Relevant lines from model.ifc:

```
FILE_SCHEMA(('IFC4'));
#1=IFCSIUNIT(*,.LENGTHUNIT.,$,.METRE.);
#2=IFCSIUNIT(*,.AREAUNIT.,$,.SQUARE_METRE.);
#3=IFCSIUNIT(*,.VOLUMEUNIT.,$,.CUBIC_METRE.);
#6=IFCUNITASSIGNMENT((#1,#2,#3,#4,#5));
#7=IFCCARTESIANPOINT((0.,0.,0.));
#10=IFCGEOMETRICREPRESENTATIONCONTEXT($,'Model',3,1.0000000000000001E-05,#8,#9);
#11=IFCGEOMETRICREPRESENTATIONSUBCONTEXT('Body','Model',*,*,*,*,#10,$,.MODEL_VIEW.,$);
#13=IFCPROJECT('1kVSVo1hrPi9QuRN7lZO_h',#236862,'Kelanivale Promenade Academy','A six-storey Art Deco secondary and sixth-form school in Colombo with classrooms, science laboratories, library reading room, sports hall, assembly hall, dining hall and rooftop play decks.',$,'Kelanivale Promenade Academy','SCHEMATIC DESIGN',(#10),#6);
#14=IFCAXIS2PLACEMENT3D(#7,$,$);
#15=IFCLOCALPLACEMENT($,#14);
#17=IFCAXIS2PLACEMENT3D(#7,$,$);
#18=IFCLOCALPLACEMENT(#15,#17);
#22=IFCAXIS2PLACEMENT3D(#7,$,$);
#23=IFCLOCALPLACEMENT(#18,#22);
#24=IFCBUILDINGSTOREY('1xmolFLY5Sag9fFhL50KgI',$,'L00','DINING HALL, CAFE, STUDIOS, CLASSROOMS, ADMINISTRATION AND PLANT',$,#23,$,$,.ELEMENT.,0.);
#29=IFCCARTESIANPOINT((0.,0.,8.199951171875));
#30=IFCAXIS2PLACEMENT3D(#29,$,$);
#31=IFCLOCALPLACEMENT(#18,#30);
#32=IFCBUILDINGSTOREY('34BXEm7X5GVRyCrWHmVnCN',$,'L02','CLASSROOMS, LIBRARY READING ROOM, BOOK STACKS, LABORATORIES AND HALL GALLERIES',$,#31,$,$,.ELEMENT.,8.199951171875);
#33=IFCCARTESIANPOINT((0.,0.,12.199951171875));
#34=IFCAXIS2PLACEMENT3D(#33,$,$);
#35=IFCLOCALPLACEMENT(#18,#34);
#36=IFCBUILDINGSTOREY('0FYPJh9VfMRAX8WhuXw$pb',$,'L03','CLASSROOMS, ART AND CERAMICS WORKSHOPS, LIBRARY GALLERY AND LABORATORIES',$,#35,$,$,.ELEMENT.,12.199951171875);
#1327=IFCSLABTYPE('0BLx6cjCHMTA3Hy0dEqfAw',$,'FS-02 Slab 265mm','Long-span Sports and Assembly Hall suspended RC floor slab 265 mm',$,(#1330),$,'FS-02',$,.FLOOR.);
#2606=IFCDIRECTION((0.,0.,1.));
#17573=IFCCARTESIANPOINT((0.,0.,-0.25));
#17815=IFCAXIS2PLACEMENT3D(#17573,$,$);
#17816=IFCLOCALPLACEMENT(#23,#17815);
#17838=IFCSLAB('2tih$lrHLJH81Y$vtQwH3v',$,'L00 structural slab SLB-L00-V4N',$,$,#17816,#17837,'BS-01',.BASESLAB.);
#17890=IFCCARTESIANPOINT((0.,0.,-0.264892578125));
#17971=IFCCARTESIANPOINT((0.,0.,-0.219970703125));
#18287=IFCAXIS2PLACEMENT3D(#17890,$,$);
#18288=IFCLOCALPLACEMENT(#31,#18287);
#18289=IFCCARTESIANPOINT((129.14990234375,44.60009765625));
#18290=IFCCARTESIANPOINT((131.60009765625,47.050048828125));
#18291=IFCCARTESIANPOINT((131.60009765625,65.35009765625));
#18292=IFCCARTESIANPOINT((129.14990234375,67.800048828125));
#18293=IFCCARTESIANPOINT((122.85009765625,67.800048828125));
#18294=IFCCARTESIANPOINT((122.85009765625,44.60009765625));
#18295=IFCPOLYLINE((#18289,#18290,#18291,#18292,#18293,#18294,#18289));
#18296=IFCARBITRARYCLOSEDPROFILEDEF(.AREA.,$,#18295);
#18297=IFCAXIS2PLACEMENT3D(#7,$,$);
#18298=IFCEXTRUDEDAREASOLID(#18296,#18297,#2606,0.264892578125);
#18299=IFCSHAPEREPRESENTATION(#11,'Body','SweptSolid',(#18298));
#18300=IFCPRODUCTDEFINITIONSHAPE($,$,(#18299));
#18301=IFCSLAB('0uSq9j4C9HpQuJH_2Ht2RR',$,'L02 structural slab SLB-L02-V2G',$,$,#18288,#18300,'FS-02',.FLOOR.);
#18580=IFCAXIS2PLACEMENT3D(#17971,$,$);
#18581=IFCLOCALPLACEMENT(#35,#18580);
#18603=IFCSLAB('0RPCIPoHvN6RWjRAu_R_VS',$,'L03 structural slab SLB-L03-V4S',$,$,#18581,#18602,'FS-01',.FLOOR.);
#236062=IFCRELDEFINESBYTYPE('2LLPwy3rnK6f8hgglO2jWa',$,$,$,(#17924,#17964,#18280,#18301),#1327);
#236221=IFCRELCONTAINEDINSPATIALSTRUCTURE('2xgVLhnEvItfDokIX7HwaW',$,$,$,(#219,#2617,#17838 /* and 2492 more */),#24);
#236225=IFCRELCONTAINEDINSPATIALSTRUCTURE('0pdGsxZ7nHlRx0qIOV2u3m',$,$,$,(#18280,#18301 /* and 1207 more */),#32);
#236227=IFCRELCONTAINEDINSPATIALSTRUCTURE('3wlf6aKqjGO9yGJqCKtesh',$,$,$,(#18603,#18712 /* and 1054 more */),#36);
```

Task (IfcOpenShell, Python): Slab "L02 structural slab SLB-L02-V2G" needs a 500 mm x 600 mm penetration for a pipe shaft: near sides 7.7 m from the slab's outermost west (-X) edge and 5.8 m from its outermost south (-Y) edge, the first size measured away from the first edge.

```python
import numpy as np
import ifcopenshell
import ifcopenshell.api.feature
import ifcopenshell.api.geometry
import ifcopenshell.api.root
import ifcopenshell.geom
import ifcopenshell.util.placement
import ifcopenshell.util.representation
import ifcopenshell.util.shape
import ifcopenshell.util.unit

model = ifcopenshell.open("model.ifc")
unit_scale = ifcopenshell.util.unit.calculate_unit_scale(model)
settings = ifcopenshell.geom.settings()


def volume(element):
    """Net volume in cubic metres, openings subtracted."""
    shape = ifcopenshell.geom.create_shape(settings, element)
    return ifcopenshell.util.shape.get_volume(shape.geometry)


slab = model.by_guid("0uSq9j4C9HpQuJH_2Ht2RR")
before = volume(slab)

# Extent in the slab's own axes, in metres. The edges named are its -X and -Y sides.
slab_shape = ifcopenshell.geom.create_shape(settings, slab)
vertices = ifcopenshell.util.shape.get_vertices(slab_shape.geometry)
x_min, y_min, bottom = vertices.min(axis=0)
top = vertices[:, 2].max()

opening = ifcopenshell.api.root.create_entity(model, ifc_class="IfcOpeningElement", name="Pipe shaft opening", predefined_type="OPENING")
context = ifcopenshell.util.representation.get_context(model, "Model", "Body", "MODEL_VIEW")
width, depth = 0.5, 0.6
outline = [(0.0, 0.0), (width, 0.0), (width, depth), (0.0, depth), (0.0, 0.0)]
# Overshoot both faces by 50 mm so the cut is clean.
shape = ifcopenshell.api.geometry.add_slab_representation(
    model, context=context, depth=top - bottom + 0.1, polyline=outline
)
ifcopenshell.api.geometry.assign_representation(model, product=opening, representation=shape)

matrix = ifcopenshell.util.placement.get_local_placement(slab.ObjectPlacement)
matrix[:, 3] = matrix @ np.append(np.array([x_min + 7.7, y_min + 5.8, bottom - 0.05]) / unit_scale, 1.0)
ifcopenshell.api.geometry.edit_object_placement(model, product=opening, matrix=matrix, is_si=False)
ifcopenshell.api.feature.add_feature(model, feature=opening, element=slab)

after = volume(slab)

print(f"slab volume {before:.3f} -> {after:.3f} m3")

model.write("model_rev.ifc")
```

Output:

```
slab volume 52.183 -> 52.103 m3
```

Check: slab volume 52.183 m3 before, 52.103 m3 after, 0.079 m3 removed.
